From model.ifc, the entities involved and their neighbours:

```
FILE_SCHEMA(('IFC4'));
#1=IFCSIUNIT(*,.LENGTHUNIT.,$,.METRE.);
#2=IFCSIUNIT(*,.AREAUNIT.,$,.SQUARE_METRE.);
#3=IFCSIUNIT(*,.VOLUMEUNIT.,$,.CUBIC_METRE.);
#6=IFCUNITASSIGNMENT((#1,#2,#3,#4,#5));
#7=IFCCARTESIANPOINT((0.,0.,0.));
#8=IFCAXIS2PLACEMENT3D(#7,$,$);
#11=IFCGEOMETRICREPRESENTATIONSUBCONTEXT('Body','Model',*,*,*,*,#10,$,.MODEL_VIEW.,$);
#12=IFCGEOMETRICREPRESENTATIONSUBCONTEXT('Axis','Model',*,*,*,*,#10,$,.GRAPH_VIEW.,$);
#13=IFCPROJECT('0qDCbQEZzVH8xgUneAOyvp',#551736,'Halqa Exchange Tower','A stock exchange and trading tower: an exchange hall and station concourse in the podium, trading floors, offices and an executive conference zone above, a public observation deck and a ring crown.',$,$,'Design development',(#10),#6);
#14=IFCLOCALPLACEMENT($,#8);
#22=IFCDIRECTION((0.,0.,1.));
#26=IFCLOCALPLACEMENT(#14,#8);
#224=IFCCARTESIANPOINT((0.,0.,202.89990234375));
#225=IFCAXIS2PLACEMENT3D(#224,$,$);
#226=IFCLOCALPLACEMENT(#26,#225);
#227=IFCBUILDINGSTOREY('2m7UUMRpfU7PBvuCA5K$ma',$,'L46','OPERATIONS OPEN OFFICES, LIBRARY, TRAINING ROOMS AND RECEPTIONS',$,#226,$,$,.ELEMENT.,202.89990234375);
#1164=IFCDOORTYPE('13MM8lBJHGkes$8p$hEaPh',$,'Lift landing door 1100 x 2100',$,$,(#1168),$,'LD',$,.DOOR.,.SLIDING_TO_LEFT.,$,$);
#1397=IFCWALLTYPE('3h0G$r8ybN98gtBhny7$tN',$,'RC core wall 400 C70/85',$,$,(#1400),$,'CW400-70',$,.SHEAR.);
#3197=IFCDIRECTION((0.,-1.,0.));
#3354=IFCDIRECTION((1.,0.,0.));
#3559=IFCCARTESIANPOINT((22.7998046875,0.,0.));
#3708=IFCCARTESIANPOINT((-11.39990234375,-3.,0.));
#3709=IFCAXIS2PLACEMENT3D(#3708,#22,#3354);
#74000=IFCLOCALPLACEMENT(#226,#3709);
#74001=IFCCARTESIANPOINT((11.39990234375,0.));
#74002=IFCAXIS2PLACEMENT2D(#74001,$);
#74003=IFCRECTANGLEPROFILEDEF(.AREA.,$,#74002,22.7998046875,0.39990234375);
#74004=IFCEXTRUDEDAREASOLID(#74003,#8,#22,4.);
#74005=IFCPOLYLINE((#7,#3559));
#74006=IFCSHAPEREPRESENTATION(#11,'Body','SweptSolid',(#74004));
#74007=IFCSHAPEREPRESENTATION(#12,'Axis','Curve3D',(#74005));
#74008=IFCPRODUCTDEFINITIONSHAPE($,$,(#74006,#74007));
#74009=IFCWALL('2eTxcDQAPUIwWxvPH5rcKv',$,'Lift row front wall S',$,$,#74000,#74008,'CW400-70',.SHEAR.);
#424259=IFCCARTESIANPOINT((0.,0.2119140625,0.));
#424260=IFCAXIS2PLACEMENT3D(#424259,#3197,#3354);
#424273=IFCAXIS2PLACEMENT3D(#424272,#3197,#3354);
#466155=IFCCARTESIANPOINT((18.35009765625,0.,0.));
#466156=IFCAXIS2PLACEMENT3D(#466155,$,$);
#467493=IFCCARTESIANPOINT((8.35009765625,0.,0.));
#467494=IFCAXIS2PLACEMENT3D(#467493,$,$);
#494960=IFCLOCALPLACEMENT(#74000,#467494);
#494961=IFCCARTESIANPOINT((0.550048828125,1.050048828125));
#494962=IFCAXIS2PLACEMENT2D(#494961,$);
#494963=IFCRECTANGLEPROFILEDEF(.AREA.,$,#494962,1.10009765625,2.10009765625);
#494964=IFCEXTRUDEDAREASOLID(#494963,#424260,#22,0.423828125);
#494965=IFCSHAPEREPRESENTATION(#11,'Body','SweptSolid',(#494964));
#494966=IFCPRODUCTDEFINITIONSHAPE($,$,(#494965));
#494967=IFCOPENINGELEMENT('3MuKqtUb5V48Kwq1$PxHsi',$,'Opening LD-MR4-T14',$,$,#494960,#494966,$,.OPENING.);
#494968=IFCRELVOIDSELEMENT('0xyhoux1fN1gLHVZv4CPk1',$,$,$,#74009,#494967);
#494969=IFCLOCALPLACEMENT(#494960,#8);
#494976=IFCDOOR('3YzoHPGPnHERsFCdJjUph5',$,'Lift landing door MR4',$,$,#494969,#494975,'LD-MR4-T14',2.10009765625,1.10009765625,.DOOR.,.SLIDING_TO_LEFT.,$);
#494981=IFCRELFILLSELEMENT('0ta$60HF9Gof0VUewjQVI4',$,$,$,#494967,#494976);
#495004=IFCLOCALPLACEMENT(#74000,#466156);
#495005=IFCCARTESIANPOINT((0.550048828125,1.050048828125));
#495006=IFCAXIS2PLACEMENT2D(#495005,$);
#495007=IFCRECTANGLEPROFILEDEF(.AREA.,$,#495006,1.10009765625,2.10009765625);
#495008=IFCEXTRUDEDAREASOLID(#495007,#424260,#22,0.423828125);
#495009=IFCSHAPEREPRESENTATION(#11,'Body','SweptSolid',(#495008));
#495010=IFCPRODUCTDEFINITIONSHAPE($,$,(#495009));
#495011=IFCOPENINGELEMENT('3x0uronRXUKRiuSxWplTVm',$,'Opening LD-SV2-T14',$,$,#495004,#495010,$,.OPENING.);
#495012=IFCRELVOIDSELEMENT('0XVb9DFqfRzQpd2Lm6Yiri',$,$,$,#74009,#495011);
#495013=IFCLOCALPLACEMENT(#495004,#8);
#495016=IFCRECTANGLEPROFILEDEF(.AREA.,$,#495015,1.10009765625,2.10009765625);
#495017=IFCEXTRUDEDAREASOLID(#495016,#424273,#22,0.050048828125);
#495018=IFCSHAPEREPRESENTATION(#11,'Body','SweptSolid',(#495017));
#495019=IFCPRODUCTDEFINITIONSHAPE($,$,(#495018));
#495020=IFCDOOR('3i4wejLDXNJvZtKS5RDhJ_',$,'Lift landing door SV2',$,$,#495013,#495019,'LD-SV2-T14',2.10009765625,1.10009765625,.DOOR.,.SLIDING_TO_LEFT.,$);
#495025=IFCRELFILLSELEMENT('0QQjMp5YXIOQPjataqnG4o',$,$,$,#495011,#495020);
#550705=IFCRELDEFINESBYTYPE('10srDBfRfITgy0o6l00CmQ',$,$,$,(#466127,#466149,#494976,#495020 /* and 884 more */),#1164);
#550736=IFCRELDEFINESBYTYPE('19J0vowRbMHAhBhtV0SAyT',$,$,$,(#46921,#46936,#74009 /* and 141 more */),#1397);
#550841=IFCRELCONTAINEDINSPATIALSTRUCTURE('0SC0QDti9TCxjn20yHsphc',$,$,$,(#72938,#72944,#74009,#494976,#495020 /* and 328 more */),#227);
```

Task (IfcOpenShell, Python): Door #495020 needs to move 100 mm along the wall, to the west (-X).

```python
import ifcopenshell
import ifcopenshell.api.geometry
import ifcopenshell.util.placement
import ifcopenshell.util.unit

model = ifcopenshell.open("model.ifc")
unit_scale = ifcopenshell.util.unit.calculate_unit_scale(model)

door = model.by_guid("3i4wejLDXNJvZtKS5RDhJ_")
opening = door.FillsVoids[0].RelatingOpeningElement
wall = opening.VoidsElements[0].RelatingBuildingElement

wall_matrix = ifcopenshell.util.placement.get_local_placement(wall.ObjectPlacement)
shift = wall_matrix[:3, 0] * -0.1 / unit_scale
before = ifcopenshell.util.placement.get_local_placement(door.ObjectPlacement)[:3, 3].copy()

# The door is placed relative to its opening, so it follows when the opening moves.
matrix = ifcopenshell.util.placement.get_local_placement(opening.ObjectPlacement)
matrix[:3, 3] += shift
ifcopenshell.api.geometry.edit_object_placement(
    model, product=opening, matrix=matrix, is_si=False, should_transform_children=True
)

after = ifcopenshell.util.placement.get_local_placement(door.ObjectPlacement)[:3, 3]
print("door moved by", (after - before).round(3) + 0.0)

model.write("model_v2.ifc")
```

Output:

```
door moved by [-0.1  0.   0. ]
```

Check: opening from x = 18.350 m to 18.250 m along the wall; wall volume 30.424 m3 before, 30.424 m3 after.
